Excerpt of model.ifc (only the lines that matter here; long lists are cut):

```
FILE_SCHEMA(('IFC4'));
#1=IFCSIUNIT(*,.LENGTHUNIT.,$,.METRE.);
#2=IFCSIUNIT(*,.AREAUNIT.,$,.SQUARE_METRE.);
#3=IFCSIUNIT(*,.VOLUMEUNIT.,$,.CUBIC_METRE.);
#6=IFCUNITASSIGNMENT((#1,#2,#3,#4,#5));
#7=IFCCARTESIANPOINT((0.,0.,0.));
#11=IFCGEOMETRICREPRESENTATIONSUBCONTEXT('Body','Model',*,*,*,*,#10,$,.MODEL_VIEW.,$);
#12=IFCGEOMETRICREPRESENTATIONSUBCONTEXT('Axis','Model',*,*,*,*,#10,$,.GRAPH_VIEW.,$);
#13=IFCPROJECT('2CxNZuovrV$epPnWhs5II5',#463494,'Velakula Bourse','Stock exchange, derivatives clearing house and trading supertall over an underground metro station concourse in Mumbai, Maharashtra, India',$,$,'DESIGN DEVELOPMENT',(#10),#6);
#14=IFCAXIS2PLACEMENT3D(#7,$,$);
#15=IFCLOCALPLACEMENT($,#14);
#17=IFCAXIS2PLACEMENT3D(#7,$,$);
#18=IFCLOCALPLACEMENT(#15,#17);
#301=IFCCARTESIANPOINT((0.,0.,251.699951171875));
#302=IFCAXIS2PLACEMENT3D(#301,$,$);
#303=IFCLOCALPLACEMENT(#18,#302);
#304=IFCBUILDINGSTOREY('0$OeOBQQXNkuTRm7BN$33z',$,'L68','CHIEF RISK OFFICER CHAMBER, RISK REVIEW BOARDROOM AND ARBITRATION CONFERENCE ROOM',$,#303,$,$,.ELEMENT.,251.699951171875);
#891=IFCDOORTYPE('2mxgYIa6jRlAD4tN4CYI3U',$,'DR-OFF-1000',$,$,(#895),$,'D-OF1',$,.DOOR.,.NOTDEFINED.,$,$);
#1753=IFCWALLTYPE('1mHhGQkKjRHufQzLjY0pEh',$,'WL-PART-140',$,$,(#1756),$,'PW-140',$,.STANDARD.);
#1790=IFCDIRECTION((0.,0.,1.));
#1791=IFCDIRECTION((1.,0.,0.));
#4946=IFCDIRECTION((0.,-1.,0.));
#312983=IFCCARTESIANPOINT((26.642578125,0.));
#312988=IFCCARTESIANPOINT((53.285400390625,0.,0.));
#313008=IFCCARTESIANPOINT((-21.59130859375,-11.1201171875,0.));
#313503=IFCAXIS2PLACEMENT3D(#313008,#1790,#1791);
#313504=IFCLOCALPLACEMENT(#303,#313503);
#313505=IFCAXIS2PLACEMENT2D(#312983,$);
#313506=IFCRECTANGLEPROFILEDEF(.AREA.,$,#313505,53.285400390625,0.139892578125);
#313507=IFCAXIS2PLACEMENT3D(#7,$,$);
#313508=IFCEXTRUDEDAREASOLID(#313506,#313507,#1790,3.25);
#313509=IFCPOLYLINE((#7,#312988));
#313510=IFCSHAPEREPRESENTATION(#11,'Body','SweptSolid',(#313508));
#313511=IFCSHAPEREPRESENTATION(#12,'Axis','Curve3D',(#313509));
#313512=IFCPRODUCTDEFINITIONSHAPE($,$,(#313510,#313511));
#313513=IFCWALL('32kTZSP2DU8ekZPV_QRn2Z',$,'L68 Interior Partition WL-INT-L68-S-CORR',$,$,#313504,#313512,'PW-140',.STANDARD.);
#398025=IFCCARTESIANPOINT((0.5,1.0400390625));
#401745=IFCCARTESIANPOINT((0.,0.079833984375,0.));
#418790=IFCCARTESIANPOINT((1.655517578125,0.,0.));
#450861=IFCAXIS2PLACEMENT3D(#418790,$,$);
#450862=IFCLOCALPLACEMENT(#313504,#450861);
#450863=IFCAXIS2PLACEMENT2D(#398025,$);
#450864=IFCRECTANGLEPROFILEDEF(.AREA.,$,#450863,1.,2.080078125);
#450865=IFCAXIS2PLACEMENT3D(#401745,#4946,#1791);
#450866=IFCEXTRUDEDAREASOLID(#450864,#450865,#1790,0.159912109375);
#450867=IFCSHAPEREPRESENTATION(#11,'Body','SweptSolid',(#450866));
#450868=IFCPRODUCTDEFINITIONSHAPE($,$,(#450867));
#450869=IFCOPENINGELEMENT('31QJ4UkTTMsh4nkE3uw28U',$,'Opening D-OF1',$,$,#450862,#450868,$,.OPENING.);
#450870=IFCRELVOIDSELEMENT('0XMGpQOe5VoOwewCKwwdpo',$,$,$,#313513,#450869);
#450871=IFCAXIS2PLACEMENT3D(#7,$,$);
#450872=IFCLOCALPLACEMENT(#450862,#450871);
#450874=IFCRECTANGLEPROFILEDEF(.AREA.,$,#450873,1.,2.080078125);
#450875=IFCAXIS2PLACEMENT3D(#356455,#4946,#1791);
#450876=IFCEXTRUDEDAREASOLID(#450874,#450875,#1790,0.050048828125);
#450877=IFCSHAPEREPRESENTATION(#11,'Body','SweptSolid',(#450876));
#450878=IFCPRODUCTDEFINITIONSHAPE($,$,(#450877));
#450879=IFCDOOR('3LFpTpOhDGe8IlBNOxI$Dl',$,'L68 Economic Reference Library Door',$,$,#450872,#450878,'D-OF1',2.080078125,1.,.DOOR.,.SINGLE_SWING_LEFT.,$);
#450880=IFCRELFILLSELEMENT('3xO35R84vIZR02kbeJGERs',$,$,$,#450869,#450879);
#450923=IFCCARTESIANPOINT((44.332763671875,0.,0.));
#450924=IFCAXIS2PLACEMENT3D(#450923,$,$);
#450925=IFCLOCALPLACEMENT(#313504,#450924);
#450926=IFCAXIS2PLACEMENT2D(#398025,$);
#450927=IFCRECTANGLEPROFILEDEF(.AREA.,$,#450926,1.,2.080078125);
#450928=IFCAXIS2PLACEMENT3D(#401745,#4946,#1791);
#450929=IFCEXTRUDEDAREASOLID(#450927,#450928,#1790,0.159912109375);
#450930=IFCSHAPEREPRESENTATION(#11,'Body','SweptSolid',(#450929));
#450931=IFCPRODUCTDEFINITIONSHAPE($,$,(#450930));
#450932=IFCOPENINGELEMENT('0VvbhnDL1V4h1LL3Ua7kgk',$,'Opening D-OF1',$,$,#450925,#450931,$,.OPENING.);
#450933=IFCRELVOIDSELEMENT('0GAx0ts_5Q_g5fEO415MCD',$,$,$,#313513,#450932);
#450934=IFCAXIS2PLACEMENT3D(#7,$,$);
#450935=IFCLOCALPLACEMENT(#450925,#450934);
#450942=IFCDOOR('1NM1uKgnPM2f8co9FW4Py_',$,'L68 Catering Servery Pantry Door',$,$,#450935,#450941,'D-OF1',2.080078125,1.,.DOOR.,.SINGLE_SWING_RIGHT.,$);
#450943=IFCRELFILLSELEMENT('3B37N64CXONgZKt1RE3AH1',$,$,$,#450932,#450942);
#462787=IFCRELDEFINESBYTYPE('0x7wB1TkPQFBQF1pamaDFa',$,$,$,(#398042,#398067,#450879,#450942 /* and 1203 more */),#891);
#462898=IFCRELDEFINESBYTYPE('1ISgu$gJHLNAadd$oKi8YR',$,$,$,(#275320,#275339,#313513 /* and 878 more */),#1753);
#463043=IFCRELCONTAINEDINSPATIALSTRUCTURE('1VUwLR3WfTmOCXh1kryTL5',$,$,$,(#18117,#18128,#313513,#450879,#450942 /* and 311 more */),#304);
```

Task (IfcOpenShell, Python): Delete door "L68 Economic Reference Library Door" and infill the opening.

```python
import ifcopenshell
import ifcopenshell.api.feature
import ifcopenshell.api.root
import ifcopenshell.geom
import ifcopenshell.util.shape

model = ifcopenshell.open("model.ifc")
settings = ifcopenshell.geom.settings()


def volume(element):
    """Net volume in cubic metres, openings subtracted."""
    shape = ifcopenshell.geom.create_shape(settings, element)
    return ifcopenshell.util.shape.get_volume(shape.geometry)


door = model.by_guid("3LFpTpOhDGe8IlBNOxI$Dl")
opening = door.FillsVoids[0].RelatingOpeningElement
wall = opening.VoidsElements[0].RelatingBuildingElement
before = volume(wall)

ifcopenshell.api.root.remove_product(model, product=door)
ifcopenshell.api.feature.remove_feature(model, feature=opening)

after = volume(wall)

print(f"wall volume {before:.3f} -> {after:.3f} m3")

model.write("model-out.ifc")
```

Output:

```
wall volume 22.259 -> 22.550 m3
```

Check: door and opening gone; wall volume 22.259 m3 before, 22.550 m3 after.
